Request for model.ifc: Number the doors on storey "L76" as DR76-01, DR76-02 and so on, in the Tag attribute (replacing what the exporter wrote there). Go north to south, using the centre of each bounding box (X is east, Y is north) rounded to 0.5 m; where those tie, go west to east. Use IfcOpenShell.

First a look at what the model holds.

```python
import ifcopenshell
import ifcopenshell.util.element
import ifcopenshell.util.placement

model = ifcopenshell.open("model.ifc")
print(model.schema)
storey = next(s for s in model.by_type("IfcBuildingStorey") if s.Name == "L76")
doors = [e for e in ifcopenshell.util.element.get_decomposition(storey) if e.is_a("IfcDoor")]
for e in sorted(doors, key=lambda e: e.id()):
    origin = ifcopenshell.util.placement.get_local_placement(e.ObjectPlacement)[:3, 3]
    print(e.id(), e.Tag, e.Name, origin.round(2) + 0.0, sep=" | ")
```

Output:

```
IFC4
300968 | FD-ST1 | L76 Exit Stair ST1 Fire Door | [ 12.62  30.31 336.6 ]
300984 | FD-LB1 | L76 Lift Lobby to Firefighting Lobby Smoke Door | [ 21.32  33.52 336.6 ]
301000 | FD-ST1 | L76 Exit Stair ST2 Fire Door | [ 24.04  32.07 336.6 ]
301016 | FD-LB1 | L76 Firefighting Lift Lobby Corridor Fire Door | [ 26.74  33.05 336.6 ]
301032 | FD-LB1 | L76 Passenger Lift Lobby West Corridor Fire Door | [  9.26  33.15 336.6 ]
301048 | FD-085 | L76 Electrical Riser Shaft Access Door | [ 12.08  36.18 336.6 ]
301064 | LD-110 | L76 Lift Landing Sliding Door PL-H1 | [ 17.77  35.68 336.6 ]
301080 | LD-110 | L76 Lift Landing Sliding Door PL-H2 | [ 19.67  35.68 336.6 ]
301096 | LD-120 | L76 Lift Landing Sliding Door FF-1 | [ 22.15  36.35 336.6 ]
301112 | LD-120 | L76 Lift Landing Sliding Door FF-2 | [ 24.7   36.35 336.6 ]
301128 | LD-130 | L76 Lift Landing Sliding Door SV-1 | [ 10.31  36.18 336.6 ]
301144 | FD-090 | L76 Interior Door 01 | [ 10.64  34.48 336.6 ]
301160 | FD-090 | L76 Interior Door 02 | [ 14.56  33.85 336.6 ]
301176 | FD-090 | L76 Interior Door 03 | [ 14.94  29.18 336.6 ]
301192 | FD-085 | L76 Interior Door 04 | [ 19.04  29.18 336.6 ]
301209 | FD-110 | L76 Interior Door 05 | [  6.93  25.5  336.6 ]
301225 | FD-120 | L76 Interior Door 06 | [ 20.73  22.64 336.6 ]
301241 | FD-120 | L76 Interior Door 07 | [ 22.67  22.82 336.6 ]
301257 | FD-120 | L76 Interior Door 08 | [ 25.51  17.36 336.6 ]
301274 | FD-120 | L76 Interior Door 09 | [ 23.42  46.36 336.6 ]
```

```python
import ifcopenshell
import ifcopenshell.geom
import ifcopenshell.util.element
import ifcopenshell.util.shape

model = ifcopenshell.open("model.ifc")
settings = ifcopenshell.geom.settings()
settings.set("use-world-coords", True)


def centre(element):
    shape = ifcopenshell.geom.create_shape(settings, element)
    return ifcopenshell.util.shape.get_bbox_centroid(shape.geometry)


storey = next(s for s in model.by_type("IfcBuildingStorey") if s.Name == "L76")
doors = [e for e in ifcopenshell.util.element.get_decomposition(storey) if e.is_a("IfcDoor")]

# Insertion points can sit at a corner or the storey origin, so sort by the geometry (in metres).
centres = {e: centre(e) for e in doors}
doors.sort(key=lambda e: (-round(centres[e][1] / 0.5), centres[e][0]))

for i, e in enumerate(doors, start=1):
    number = f"DR76-{i:02d}"
    e.Tag = number
    print(e.id(), number)

model.write("model_v2.ifc")
```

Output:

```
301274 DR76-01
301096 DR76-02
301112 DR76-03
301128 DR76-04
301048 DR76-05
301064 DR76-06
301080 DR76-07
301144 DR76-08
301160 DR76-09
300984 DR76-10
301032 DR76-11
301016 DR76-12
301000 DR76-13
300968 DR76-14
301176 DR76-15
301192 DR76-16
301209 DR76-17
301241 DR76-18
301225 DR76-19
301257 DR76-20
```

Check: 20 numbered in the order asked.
